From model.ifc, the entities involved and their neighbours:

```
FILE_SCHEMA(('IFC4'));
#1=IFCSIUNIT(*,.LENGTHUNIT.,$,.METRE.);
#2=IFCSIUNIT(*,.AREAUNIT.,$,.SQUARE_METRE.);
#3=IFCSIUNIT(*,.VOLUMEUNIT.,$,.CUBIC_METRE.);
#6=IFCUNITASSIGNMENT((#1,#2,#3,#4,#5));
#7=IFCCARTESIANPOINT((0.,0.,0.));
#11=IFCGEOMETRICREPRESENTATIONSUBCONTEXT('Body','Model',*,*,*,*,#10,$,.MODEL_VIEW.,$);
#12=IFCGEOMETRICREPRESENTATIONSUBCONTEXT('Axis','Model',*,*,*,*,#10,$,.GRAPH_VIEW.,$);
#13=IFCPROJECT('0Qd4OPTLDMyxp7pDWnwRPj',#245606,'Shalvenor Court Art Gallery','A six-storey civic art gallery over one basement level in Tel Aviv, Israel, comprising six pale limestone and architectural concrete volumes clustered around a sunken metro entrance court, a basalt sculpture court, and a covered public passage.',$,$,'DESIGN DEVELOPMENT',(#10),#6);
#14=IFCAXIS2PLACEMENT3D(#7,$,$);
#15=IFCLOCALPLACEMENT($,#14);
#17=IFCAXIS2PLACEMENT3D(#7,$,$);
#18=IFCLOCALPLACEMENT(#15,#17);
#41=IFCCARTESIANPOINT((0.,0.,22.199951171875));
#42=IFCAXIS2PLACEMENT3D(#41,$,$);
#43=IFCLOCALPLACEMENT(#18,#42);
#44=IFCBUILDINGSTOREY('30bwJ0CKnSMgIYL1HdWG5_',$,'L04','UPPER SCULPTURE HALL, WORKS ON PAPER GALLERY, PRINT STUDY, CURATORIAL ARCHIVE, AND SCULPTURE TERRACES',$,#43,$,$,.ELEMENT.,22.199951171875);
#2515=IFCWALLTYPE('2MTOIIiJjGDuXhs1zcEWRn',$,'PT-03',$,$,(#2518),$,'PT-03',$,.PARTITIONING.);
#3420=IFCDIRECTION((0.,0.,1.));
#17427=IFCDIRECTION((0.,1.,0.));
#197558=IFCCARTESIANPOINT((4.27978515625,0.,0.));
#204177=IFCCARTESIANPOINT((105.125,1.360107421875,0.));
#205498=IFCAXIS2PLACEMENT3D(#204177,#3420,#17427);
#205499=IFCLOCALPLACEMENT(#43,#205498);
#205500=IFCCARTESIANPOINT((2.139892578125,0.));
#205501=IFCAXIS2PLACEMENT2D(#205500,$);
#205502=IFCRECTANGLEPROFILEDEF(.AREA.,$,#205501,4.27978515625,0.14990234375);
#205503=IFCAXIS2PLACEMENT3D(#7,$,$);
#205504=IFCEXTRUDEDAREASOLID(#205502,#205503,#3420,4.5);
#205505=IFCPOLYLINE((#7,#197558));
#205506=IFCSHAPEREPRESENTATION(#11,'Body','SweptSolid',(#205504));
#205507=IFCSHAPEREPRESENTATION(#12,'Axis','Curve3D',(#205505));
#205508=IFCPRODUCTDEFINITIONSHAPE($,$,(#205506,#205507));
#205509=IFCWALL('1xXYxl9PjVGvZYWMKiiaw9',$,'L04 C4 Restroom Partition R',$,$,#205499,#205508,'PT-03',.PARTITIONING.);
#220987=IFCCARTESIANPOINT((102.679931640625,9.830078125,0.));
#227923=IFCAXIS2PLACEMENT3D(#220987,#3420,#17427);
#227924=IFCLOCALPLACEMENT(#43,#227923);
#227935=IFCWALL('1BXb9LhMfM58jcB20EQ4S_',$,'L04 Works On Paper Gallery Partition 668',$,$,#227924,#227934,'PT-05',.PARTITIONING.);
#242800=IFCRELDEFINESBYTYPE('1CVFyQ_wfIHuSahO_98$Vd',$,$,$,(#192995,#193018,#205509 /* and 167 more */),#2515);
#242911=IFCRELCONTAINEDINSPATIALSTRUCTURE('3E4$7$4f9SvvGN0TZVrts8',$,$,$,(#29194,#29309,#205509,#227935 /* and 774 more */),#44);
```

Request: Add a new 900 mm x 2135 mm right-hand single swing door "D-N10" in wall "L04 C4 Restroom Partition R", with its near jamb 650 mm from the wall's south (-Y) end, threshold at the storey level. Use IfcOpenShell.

```python
import numpy as np
import ifcopenshell
import ifcopenshell.api.feature
import ifcopenshell.api.geometry
import ifcopenshell.api.root
import ifcopenshell.api.spatial
import ifcopenshell.geom
import ifcopenshell.util.element
import ifcopenshell.util.placement
import ifcopenshell.util.representation
import ifcopenshell.util.shape
import ifcopenshell.util.unit

model = ifcopenshell.open("model.ifc")
unit_scale = ifcopenshell.util.unit.calculate_unit_scale(model)
settings = ifcopenshell.geom.settings()


def volume(element):
    """Net volume in cubic metres, openings subtracted."""
    shape = ifcopenshell.geom.create_shape(settings, element)
    return ifcopenshell.util.shape.get_volume(shape.geometry)


wall = model.by_id(205509)
storey = ifcopenshell.util.element.get_container(wall, ifc_class="IfcBuildingStorey")
context = ifcopenshell.util.representation.get_context(model, "Model", "Body", "MODEL_VIEW")
before = volume(wall)

width, height, from_end, sill = 0.9, 2.135, 0.65, 0.0  # metres

# The wall runs along its own X axis, and the end named is its -X end.
wall_shape = ifcopenshell.geom.create_shape(settings, wall)
x, y, z = ifcopenshell.util.shape.get_vertices(wall_shape.geometry).T
start = x.min() + from_end
face, thickness = float(y.min()), float(y.max() - y.min())
wall_matrix = ifcopenshell.util.placement.get_local_placement(wall.ObjectPlacement)
level = ifcopenshell.util.placement.get_local_placement(storey.ObjectPlacement)[2, 3]


def in_wall(x, y):
    """Placement at x, y metres in the wall's axes, at sill height."""
    matrix = wall_matrix.copy()
    matrix[:, 3] = wall_matrix @ np.array([x / unit_scale, y / unit_scale, 0.0, 1.0])
    matrix[2, 3] = level + sill / unit_scale
    return matrix


# Opening: a box that overshoots both wall faces by 50 mm.
opening = ifcopenshell.api.root.create_entity(model, ifc_class="IfcOpeningElement", predefined_type="OPENING")
box = ifcopenshell.api.geometry.add_wall_representation(
    model, context=context, length=width, height=height, thickness=thickness + 0.1
)
ifcopenshell.api.geometry.assign_representation(model, product=opening, representation=box)
ifcopenshell.api.geometry.edit_object_placement(model, product=opening, matrix=in_wall(start, face - 0.05), is_si=False)
ifcopenshell.api.feature.add_feature(model, feature=opening, element=wall)

door = ifcopenshell.api.root.create_entity(model, ifc_class="IfcDoor", name="D-N10", predefined_type="DOOR")
door.OverallWidth, door.OverallHeight = width / unit_scale, height / unit_scale
door.OperationType = "SINGLE_SWING_RIGHT"
body = ifcopenshell.api.geometry.add_door_representation(
    model,
    context=context,
    overall_width=door.OverallWidth,
    overall_height=door.OverallHeight,
    operation_type="SINGLE_SWING_RIGHT",
    lining_properties={"LiningDepth": thickness / unit_scale, "ThresholdDepth": thickness / unit_scale},
)
ifcopenshell.api.geometry.assign_representation(model, product=door, representation=body)
ifcopenshell.api.spatial.assign_container(model, products=[door], relating_structure=storey)
ifcopenshell.api.feature.add_filling(model, opening=opening, element=door)

# The lining spans the wall, so the door starts at the wall face.
ifcopenshell.api.geometry.edit_object_placement(model, product=door, matrix=in_wall(start, face), is_si=False)

after = volume(wall)

print(f"wall volume {before:.3f} -> {after:.3f} m3")

model.write("model_v2.ifc")
```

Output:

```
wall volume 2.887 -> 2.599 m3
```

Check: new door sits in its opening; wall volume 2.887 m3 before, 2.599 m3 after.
